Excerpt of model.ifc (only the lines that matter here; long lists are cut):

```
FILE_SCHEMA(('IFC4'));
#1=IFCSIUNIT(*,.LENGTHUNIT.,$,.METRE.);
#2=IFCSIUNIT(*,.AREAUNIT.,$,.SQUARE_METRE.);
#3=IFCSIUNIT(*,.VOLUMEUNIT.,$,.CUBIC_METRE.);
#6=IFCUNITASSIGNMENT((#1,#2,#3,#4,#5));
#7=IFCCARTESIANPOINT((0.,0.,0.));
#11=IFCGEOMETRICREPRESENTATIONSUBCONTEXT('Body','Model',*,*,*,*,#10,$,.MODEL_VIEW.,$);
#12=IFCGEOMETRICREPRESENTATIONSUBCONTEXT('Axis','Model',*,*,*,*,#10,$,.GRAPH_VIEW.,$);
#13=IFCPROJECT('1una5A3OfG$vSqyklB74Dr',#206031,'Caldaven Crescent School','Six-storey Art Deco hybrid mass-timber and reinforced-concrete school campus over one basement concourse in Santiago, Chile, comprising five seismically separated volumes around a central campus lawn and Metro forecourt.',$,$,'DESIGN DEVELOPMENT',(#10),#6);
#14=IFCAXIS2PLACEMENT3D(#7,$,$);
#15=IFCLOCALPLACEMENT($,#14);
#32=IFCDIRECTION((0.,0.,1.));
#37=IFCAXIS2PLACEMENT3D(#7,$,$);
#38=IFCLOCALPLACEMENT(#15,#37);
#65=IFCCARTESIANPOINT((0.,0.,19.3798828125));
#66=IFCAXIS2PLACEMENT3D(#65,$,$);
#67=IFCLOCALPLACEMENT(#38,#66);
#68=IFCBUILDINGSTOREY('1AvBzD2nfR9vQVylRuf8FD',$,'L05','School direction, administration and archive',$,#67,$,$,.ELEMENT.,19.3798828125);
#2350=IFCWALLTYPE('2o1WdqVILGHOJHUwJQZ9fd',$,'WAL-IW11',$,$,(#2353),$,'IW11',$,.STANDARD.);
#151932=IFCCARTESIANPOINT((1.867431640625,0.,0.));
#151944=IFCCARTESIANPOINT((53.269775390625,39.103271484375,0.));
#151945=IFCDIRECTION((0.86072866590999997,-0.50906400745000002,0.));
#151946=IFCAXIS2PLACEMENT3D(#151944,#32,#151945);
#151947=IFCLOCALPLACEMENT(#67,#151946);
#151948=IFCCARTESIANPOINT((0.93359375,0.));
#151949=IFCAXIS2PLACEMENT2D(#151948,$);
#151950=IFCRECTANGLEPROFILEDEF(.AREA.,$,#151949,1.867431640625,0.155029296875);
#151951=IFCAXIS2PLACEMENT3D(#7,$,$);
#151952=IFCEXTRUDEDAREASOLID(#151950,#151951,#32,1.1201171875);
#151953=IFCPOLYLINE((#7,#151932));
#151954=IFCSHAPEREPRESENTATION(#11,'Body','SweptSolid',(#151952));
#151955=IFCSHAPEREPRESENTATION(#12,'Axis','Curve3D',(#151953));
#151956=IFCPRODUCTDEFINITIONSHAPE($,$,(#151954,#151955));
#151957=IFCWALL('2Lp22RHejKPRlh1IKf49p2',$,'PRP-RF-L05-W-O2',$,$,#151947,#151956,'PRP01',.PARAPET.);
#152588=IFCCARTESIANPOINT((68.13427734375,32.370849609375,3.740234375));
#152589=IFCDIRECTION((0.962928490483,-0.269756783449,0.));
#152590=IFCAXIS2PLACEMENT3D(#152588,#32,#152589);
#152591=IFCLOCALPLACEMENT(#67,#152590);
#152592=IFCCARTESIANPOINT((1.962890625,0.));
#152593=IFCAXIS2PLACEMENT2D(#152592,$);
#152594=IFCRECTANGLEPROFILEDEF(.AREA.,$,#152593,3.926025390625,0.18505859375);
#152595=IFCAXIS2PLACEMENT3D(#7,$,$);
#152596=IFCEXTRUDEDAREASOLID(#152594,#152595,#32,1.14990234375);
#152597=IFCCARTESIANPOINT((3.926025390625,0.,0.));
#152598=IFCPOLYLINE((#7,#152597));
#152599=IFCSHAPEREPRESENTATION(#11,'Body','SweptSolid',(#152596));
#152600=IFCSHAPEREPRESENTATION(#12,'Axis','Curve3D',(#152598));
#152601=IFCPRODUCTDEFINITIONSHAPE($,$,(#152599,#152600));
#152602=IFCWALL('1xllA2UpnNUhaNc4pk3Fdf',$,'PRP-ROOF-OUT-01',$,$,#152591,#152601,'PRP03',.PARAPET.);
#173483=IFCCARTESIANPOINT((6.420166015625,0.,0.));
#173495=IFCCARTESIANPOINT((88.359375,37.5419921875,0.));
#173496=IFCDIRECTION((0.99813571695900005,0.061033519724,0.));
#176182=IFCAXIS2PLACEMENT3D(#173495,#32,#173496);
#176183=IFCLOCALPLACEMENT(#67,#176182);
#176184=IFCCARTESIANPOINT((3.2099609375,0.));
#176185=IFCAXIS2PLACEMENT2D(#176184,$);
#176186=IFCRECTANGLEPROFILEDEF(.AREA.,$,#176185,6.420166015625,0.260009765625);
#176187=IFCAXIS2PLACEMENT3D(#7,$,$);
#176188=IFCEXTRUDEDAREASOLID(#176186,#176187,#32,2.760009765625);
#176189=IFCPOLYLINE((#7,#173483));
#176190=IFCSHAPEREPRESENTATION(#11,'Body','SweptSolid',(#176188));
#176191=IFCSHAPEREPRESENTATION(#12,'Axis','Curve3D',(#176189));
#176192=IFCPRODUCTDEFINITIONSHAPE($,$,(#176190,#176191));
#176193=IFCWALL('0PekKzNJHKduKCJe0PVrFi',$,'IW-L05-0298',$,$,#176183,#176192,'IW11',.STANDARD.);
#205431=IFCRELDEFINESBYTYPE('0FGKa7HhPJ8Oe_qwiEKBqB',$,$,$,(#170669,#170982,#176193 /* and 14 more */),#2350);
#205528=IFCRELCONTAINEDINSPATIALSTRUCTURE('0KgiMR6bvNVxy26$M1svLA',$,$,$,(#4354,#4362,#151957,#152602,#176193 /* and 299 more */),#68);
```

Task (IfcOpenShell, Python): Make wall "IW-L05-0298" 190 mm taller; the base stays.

```python
import ifcopenshell
import ifcopenshell.geom
import ifcopenshell.util.representation
import ifcopenshell.util.shape
import ifcopenshell.util.unit

model = ifcopenshell.open("model.ifc")
unit_scale = ifcopenshell.util.unit.calculate_unit_scale(model)
settings = ifcopenshell.geom.settings()


def volume(element):
    """Net volume in cubic metres, openings subtracted."""
    shape = ifcopenshell.geom.create_shape(settings, element)
    return ifcopenshell.util.shape.get_volume(shape.geometry)


wall = model.by_guid("0PekKzNJHKduKCJe0PVrFi")
before = volume(wall)

body = ifcopenshell.util.representation.get_representation(wall, "Model", "Body")
solid = body.Items[0]
old_height = solid.Depth
solid.Depth += 0.19 / unit_scale
after = volume(wall)

print(f"height {old_height:g} -> {solid.Depth:g}, volume {before:.3f} -> {after:.3f} m3")

model.write("model_edited.ifc")
```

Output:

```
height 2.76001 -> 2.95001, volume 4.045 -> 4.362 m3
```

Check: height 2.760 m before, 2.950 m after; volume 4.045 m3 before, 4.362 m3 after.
